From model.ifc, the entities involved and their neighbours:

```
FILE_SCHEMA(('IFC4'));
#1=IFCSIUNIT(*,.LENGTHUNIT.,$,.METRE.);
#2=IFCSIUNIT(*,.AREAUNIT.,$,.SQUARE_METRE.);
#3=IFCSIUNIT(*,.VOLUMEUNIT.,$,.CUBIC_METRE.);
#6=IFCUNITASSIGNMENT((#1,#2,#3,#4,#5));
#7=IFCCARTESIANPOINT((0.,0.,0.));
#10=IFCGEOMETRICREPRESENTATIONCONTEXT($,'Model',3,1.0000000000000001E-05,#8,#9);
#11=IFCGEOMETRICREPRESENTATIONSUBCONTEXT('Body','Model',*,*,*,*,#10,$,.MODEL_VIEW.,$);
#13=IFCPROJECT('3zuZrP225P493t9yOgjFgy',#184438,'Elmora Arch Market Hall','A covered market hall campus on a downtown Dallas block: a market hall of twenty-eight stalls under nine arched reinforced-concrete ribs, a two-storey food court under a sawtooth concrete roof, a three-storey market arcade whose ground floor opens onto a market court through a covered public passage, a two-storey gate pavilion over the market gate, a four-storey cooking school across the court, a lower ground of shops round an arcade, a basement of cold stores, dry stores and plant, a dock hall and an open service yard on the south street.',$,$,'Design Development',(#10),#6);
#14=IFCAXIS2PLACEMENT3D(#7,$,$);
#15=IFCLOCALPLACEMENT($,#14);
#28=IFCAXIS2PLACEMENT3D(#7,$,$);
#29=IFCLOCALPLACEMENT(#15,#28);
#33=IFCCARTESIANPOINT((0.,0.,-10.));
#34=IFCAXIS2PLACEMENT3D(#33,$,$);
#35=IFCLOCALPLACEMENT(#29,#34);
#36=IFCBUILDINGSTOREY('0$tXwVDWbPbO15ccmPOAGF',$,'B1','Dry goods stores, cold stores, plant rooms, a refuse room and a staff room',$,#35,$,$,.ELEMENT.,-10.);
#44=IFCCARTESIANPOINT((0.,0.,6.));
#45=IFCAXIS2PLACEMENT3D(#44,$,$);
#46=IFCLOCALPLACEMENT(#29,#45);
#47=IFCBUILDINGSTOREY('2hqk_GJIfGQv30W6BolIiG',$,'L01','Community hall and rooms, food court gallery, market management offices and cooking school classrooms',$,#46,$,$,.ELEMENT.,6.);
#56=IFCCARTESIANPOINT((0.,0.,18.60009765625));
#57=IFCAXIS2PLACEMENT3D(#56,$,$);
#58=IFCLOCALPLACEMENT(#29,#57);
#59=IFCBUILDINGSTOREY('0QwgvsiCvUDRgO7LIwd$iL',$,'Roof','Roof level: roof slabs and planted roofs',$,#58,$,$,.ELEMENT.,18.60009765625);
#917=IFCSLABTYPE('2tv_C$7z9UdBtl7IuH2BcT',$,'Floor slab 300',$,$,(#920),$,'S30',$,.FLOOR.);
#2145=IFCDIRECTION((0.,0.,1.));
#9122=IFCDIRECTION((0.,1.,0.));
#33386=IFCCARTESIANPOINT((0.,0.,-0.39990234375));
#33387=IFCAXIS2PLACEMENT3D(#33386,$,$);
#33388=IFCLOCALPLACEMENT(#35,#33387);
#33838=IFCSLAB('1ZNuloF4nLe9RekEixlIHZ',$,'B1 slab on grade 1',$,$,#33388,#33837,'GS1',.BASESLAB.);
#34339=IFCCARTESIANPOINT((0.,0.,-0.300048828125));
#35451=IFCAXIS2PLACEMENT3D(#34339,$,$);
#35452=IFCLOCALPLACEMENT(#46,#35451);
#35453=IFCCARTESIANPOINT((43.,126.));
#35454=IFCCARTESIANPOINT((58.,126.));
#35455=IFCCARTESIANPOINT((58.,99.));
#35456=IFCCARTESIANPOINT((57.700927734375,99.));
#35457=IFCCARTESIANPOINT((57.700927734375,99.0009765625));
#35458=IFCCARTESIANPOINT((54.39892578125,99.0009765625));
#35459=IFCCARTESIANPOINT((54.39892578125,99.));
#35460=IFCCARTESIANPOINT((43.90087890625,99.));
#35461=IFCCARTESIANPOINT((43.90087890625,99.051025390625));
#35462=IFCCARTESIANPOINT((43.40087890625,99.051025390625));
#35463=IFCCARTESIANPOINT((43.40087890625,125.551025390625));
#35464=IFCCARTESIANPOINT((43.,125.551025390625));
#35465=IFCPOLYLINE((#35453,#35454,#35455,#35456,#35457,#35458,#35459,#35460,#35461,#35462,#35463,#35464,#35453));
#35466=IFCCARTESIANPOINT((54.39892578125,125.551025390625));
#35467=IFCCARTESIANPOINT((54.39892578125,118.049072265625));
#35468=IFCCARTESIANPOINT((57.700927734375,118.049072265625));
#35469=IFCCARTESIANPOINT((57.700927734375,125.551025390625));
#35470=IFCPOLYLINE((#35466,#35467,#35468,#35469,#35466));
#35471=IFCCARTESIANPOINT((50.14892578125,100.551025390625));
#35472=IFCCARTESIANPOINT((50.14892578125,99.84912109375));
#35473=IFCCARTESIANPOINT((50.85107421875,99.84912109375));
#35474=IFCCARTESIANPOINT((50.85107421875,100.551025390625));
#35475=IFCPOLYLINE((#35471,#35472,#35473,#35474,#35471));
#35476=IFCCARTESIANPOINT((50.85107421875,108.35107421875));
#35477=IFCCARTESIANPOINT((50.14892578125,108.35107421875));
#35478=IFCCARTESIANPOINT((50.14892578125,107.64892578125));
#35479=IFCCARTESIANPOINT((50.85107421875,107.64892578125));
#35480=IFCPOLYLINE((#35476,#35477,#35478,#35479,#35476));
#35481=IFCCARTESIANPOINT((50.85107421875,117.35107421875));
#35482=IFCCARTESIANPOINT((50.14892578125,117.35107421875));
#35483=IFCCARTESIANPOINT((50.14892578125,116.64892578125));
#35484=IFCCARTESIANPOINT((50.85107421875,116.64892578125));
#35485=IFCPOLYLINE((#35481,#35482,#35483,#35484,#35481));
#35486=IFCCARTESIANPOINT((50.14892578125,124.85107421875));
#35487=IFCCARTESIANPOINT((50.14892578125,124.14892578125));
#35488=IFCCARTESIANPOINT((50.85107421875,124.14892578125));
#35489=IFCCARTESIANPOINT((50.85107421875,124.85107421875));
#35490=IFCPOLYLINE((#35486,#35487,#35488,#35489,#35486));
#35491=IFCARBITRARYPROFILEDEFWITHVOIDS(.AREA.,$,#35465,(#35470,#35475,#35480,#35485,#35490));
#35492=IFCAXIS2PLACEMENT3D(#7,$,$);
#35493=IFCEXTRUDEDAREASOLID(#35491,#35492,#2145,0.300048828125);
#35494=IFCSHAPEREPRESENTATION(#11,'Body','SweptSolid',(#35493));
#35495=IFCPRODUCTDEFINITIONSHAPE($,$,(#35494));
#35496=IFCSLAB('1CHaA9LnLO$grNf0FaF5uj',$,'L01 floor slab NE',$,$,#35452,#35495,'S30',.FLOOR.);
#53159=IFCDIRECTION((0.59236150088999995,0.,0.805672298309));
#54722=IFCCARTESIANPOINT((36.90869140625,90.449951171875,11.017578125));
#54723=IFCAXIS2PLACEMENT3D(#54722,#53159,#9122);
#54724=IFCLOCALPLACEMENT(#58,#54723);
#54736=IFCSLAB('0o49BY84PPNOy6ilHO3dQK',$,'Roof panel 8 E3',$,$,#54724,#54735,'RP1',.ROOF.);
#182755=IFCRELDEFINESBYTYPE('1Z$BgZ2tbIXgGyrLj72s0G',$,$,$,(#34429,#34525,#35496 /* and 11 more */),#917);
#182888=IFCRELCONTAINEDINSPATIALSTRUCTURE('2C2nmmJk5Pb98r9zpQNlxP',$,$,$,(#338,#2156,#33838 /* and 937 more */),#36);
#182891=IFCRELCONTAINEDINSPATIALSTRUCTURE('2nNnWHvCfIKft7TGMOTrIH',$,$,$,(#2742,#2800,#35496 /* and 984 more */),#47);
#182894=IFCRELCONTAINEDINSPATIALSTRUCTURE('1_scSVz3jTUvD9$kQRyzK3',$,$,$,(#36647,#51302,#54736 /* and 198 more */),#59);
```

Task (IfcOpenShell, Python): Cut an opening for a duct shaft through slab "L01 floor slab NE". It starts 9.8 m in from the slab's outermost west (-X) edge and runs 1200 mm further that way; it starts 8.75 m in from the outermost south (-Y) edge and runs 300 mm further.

```python
import numpy as np
import ifcopenshell
import ifcopenshell.api.feature
import ifcopenshell.api.geometry
import ifcopenshell.api.root
import ifcopenshell.geom
import ifcopenshell.util.placement
import ifcopenshell.util.representation
import ifcopenshell.util.shape
import ifcopenshell.util.unit

model = ifcopenshell.open("model.ifc")
unit_scale = ifcopenshell.util.unit.calculate_unit_scale(model)
settings = ifcopenshell.geom.settings()


def volume(element):
    """Net volume in cubic metres, openings subtracted."""
    shape = ifcopenshell.geom.create_shape(settings, element)
    return ifcopenshell.util.shape.get_volume(shape.geometry)


slab = model.by_guid("1CHaA9LnLO$grNf0FaF5uj")
before = volume(slab)

# Extent in the slab's own axes, in metres. The edges named are its -X and -Y sides.
slab_shape = ifcopenshell.geom.create_shape(settings, slab)
vertices = ifcopenshell.util.shape.get_vertices(slab_shape.geometry)
x_min, y_min, bottom = vertices.min(axis=0)
top = vertices[:, 2].max()

opening = ifcopenshell.api.root.create_entity(model, ifc_class="IfcOpeningElement", name="Duct shaft opening", predefined_type="OPENING")
context = ifcopenshell.util.representation.get_context(model, "Model", "Body", "MODEL_VIEW")
width, depth = 1.2, 0.3
outline = [(0.0, 0.0), (width, 0.0), (width, depth), (0.0, depth), (0.0, 0.0)]
# Overshoot both faces by 50 mm so the cut is clean.
shape = ifcopenshell.api.geometry.add_slab_representation(
    model, context=context, depth=top - bottom + 0.1, polyline=outline
)
ifcopenshell.api.geometry.assign_representation(model, product=opening, representation=shape)

matrix = ifcopenshell.util.placement.get_local_placement(slab.ObjectPlacement)
matrix[:, 3] = matrix @ np.append(np.array([x_min + 9.8, y_min + 8.75, bottom - 0.05]) / unit_scale, 1.0)
ifcopenshell.api.geometry.edit_object_placement(model, product=opening, matrix=matrix, is_si=False)
ifcopenshell.api.feature.add_feature(model, feature=opening, element=slab)

after = volume(slab)

print(f"slab volume {before:.3f} -> {after:.3f} m3")

model.write("model_v2.ifc")
```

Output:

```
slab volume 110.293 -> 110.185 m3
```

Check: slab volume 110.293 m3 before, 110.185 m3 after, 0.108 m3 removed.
